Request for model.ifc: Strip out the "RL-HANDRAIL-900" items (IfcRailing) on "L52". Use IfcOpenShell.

First a look at what the model holds.

```python
import ifcopenshell
import ifcopenshell.util.element

model = ifcopenshell.open("model.ifc")
print(model.schema)
storey = next(s for s in model.by_type("IfcBuildingStorey") if s.Name == "L52")
railings = [e for e in ifcopenshell.util.element.get_decomposition(storey) if e.is_a("IfcRailing")]
seen = {}
for e in railings:
    element_type = ifcopenshell.util.element.get_type(e)
    name = element_type.Name if element_type not in (None, e) else None
    seen[name] = seen.get(name, 0) + 1
for name, count in sorted(seen.items(), key=str):
    print(count, "x", name)
```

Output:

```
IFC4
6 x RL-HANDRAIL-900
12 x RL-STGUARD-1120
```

```python
import ifcopenshell
import ifcopenshell.api.root
import ifcopenshell.util.element

model = ifcopenshell.open("model.ifc")

storey = next(s for s in model.by_type("IfcBuildingStorey") if s.Name == "L52")
railings = [e for e in ifcopenshell.util.element.get_decomposition(storey) if e.is_a("IfcRailing")]
targets = [e for e in railings if (t := ifcopenshell.util.element.get_type(e)) not in (None, e) and t.Name == "RL-HANDRAIL-900"]

for e in targets:
    ifcopenshell.api.root.remove_product(model, product=e)
print(len(targets), "removed")

model.write("model-out.ifc")
```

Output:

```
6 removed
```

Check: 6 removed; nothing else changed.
